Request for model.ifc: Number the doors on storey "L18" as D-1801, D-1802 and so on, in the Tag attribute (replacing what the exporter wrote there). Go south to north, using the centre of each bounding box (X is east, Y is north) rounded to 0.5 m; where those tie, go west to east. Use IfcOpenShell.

First a look at what the model holds.

```python
import ifcopenshell
import ifcopenshell.util.element
import ifcopenshell.util.placement

model = ifcopenshell.open("model.ifc")
print(model.schema)
storey = next(s for s in model.by_type("IfcBuildingStorey") if s.Name == "L18")
doors = [e for e in ifcopenshell.util.element.get_decomposition(storey) if e.is_a("IfcDoor")]
for e in sorted(doors, key=lambda e: e.id()):
    origin = ifcopenshell.util.placement.get_local_placement(e.ObjectPlacement)[:3, 3]
    print(e.id(), e.Tag, e.Name, origin.round(2) + 0.0, sep=" | ")
```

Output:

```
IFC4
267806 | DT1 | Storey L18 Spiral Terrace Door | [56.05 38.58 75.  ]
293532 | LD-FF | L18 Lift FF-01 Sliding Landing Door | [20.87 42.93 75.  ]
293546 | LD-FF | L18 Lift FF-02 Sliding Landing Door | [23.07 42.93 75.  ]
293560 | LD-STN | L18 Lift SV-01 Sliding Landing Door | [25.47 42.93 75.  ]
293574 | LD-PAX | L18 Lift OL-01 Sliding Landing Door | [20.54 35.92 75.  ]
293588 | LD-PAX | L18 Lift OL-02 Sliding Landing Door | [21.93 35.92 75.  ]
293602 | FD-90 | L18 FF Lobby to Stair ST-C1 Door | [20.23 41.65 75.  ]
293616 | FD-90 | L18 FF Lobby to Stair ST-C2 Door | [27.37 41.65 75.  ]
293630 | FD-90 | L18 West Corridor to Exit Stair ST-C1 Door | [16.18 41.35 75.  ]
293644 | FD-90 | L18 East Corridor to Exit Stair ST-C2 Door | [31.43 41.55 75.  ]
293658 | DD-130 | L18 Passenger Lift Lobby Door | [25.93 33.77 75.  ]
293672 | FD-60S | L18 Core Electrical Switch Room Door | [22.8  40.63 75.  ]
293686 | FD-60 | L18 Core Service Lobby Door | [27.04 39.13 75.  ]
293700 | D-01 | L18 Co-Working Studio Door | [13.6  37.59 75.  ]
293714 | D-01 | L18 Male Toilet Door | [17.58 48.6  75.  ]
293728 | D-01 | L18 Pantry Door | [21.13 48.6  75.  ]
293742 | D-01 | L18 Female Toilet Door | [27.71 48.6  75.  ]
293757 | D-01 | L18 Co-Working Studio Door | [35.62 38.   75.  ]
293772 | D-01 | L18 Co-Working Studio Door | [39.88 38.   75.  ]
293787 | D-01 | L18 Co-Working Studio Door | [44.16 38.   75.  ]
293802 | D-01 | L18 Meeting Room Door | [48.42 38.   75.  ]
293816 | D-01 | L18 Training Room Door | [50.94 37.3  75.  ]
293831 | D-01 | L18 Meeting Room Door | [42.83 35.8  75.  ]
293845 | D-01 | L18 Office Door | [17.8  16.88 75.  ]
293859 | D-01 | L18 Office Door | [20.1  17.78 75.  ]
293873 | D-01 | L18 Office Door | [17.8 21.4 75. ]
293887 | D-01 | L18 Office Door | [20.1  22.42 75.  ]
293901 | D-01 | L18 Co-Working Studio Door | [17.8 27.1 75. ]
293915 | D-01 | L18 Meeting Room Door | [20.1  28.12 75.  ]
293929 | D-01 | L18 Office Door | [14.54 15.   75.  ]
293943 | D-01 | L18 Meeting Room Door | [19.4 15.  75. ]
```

```python
import ifcopenshell
import ifcopenshell.geom
import ifcopenshell.util.element
import ifcopenshell.util.shape

model = ifcopenshell.open("model.ifc")
settings = ifcopenshell.geom.settings()
settings.set("use-world-coords", True)


def centre(element):
    shape = ifcopenshell.geom.create_shape(settings, element)
    return ifcopenshell.util.shape.get_bbox_centroid(shape.geometry)


storey = next(s for s in model.by_type("IfcBuildingStorey") if s.Name == "L18")
doors = [e for e in ifcopenshell.util.element.get_decomposition(storey) if e.is_a("IfcDoor")]

# Insertion points can sit at a corner or the storey origin, so sort by the geometry (in metres).
centres = {e: centre(e) for e in doors}
doors.sort(key=lambda e: (round(centres[e][1] / 0.5), centres[e][0]))

for i, e in enumerate(doors, start=1):
    number = f"D-18{i:02d}"
    e.Tag = number
    print(e.id(), number)

model.write("model_edited.ifc")
```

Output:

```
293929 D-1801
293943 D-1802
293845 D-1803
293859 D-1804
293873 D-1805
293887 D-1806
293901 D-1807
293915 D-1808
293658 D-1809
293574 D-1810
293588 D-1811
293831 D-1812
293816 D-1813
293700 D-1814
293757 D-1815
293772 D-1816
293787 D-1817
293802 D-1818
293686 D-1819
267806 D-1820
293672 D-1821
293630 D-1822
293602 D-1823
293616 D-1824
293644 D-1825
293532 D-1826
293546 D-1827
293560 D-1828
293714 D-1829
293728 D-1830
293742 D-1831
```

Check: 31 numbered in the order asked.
